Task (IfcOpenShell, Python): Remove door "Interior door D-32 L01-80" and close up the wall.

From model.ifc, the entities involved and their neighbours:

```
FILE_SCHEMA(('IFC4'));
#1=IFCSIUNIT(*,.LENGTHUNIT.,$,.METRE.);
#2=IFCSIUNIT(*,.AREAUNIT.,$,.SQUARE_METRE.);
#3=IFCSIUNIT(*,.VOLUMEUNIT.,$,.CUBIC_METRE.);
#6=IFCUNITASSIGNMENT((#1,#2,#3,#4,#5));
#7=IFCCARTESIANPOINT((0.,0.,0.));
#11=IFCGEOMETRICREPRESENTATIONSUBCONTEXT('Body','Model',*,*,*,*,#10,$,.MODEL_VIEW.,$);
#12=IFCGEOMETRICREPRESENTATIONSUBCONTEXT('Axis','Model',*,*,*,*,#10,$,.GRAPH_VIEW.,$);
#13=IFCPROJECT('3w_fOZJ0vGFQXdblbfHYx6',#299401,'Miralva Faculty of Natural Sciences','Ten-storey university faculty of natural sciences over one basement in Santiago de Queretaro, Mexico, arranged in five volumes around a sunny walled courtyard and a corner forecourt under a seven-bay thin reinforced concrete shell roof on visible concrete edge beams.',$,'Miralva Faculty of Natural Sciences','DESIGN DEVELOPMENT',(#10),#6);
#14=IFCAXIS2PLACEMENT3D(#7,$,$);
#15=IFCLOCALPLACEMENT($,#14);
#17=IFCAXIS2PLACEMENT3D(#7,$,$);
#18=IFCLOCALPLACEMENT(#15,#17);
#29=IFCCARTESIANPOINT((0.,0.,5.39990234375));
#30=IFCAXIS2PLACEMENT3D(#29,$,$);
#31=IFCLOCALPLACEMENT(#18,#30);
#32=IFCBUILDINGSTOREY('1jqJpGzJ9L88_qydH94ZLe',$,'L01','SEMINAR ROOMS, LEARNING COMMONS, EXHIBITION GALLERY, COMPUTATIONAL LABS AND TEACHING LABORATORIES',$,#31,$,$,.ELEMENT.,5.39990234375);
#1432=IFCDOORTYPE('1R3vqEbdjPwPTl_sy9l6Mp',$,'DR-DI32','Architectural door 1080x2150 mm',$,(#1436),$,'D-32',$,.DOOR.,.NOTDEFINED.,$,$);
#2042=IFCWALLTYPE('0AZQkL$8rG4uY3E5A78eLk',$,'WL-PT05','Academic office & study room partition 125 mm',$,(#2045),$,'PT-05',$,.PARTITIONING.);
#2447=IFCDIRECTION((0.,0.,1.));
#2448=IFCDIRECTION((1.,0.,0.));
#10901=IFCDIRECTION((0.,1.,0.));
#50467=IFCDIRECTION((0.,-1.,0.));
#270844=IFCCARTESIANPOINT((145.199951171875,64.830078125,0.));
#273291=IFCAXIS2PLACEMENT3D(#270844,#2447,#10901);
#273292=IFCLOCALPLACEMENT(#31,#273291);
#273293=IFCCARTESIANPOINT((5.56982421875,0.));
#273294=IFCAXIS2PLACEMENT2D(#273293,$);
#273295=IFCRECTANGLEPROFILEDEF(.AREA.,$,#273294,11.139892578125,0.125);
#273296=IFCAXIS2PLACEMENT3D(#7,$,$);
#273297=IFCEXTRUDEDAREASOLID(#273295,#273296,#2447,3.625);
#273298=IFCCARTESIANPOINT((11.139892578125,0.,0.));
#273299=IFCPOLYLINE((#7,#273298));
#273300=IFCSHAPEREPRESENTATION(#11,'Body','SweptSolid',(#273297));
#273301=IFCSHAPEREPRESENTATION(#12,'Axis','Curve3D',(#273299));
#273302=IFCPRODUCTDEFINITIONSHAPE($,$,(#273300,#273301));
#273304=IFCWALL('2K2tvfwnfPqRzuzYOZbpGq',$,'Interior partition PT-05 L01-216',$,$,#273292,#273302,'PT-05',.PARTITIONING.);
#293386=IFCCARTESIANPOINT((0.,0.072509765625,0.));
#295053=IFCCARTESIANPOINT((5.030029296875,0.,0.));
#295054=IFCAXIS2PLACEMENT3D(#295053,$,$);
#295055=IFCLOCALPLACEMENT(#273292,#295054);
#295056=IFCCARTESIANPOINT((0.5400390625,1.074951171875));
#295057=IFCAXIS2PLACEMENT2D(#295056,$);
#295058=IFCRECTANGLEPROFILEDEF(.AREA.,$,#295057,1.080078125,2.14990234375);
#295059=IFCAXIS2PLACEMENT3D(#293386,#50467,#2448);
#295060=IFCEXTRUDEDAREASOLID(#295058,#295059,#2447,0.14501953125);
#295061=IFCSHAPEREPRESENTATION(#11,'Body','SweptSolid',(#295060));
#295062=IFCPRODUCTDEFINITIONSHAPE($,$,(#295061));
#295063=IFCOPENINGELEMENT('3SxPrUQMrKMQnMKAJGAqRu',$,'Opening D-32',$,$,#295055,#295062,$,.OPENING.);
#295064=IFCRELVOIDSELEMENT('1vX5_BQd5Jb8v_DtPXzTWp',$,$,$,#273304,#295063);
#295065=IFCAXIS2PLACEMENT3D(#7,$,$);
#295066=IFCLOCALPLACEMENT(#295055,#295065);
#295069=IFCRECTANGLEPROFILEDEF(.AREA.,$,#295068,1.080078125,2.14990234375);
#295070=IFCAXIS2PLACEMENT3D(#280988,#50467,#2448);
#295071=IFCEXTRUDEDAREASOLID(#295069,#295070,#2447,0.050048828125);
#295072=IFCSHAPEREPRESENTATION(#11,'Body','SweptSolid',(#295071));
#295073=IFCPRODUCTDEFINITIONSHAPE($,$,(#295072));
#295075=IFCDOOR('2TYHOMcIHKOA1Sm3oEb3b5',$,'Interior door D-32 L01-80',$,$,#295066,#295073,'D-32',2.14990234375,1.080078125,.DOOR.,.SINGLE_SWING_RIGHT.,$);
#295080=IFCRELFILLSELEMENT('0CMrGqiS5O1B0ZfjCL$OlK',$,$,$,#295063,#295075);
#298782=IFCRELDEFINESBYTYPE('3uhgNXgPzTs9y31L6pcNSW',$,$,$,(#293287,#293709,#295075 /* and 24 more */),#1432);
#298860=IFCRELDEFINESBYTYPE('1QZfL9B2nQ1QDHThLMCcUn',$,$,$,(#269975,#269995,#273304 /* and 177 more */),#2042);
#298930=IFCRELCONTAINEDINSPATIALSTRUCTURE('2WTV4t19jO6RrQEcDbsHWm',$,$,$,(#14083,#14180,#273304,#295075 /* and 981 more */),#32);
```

```python
import ifcopenshell
import ifcopenshell.api.feature
import ifcopenshell.api.root
import ifcopenshell.geom
import ifcopenshell.util.shape

model = ifcopenshell.open("model.ifc")
settings = ifcopenshell.geom.settings()


def volume(element):
    """Net volume in cubic metres, openings subtracted."""
    shape = ifcopenshell.geom.create_shape(settings, element)
    return ifcopenshell.util.shape.get_volume(shape.geometry)


door = model.by_guid("2TYHOMcIHKOA1Sm3oEb3b5")
opening = door.FillsVoids[0].RelatingOpeningElement
wall = opening.VoidsElements[0].RelatingBuildingElement
before = volume(wall)

ifcopenshell.api.root.remove_product(model, product=door)
ifcopenshell.api.feature.remove_feature(model, feature=opening)

after = volume(wall)

print(f"wall volume {before:.3f} -> {after:.3f} m3")

model.write("model_v2.ifc")
```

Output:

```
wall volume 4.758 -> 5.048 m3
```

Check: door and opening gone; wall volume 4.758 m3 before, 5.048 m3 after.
